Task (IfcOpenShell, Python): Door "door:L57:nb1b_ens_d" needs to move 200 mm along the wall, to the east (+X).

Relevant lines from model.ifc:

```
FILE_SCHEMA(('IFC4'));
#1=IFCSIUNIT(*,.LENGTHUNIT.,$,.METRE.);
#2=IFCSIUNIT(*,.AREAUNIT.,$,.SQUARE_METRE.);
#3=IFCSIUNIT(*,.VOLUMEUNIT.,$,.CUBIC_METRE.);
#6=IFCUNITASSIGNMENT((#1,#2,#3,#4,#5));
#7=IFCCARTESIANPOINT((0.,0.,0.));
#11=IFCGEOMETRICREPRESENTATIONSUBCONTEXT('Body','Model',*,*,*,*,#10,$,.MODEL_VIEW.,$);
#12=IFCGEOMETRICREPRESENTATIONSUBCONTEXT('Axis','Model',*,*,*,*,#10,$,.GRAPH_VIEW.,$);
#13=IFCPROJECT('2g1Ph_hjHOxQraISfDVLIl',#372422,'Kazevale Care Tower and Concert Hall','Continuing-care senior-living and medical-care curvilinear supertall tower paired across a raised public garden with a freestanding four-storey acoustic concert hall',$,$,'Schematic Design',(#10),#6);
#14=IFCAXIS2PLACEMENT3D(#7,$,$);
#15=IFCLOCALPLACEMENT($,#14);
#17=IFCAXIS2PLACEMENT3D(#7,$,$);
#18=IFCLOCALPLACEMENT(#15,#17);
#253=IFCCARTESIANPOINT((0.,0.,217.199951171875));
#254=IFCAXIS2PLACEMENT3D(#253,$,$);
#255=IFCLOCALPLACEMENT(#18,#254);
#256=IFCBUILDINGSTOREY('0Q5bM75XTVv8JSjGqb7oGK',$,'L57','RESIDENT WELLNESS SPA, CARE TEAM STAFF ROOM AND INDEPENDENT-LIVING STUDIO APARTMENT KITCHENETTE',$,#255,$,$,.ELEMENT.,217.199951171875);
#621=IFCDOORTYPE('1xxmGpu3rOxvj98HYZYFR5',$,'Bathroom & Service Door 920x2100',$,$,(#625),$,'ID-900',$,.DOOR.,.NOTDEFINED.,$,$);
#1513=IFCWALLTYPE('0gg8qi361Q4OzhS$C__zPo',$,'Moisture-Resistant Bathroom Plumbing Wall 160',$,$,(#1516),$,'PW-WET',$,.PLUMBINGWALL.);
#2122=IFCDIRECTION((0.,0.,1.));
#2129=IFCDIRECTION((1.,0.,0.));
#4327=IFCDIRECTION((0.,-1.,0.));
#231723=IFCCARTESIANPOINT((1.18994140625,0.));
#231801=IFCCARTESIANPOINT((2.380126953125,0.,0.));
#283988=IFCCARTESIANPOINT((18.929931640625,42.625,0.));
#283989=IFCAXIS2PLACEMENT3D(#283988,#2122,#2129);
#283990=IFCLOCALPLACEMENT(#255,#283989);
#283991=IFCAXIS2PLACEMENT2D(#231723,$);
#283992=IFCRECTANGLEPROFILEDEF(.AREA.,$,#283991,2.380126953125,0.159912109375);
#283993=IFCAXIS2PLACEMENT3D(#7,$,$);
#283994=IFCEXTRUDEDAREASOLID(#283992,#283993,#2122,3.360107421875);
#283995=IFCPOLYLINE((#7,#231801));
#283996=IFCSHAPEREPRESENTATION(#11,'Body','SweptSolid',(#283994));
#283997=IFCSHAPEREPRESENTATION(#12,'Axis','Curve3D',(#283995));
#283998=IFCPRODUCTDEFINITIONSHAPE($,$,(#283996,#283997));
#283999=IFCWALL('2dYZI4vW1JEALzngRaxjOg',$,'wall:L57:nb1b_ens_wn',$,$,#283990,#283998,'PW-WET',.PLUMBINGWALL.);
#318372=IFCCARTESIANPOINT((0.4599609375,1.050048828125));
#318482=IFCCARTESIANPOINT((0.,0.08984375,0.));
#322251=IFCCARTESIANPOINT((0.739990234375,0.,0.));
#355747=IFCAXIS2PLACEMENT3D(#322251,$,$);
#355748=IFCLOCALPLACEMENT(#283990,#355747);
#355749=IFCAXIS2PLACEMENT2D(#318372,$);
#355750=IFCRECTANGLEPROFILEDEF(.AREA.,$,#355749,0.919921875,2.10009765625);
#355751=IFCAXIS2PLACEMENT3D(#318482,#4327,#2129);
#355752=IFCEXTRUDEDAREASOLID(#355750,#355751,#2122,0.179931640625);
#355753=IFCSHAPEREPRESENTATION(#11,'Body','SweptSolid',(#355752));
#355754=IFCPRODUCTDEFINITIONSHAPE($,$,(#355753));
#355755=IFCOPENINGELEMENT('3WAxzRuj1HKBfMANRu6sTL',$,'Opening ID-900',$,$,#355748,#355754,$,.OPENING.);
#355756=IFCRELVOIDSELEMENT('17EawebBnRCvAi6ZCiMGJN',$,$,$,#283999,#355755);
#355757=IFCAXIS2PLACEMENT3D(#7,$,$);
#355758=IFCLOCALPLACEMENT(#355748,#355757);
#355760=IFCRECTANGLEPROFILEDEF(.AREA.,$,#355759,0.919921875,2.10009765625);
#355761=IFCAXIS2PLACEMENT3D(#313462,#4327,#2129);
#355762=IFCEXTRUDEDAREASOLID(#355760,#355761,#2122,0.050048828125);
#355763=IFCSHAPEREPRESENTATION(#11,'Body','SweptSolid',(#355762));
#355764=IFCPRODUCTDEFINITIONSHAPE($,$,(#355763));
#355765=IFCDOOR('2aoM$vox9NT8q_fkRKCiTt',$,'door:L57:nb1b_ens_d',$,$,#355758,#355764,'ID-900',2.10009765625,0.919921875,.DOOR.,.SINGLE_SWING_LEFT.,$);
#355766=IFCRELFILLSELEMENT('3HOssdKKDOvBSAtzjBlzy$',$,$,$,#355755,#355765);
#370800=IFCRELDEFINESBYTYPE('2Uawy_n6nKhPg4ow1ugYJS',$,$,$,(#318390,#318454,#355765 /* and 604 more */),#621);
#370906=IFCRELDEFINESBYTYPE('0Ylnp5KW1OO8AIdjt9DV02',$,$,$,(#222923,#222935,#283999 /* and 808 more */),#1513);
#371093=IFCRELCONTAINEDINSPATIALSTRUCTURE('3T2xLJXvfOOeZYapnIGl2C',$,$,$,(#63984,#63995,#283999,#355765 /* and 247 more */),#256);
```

```python
import ifcopenshell
import ifcopenshell.api.geometry
import ifcopenshell.util.placement

model = ifcopenshell.open("model.ifc")

door = model.by_guid("2aoM$vox9NT8q_fkRKCiTt")
opening = door.FillsVoids[0].RelatingOpeningElement
wall = opening.VoidsElements[0].RelatingBuildingElement

wall_matrix = ifcopenshell.util.placement.get_local_placement(wall.ObjectPlacement)
shift = wall_matrix[:3, 0] * 0.2
before = ifcopenshell.util.placement.get_local_placement(door.ObjectPlacement)[:3, 3].copy()

# The door is placed relative to its opening, so it follows when the opening moves.
matrix = ifcopenshell.util.placement.get_local_placement(opening.ObjectPlacement)
matrix[:3, 3] += shift
ifcopenshell.api.geometry.edit_object_placement(
    model, product=opening, matrix=matrix, is_si=False, should_transform_children=True
)

after = ifcopenshell.util.placement.get_local_placement(door.ObjectPlacement)[:3, 3]
print("door moved by", (after - before).round(3) + 0.0)

model.write("model_v2.ifc")
```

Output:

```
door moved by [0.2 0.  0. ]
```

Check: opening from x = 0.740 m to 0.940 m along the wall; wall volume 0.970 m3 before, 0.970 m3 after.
